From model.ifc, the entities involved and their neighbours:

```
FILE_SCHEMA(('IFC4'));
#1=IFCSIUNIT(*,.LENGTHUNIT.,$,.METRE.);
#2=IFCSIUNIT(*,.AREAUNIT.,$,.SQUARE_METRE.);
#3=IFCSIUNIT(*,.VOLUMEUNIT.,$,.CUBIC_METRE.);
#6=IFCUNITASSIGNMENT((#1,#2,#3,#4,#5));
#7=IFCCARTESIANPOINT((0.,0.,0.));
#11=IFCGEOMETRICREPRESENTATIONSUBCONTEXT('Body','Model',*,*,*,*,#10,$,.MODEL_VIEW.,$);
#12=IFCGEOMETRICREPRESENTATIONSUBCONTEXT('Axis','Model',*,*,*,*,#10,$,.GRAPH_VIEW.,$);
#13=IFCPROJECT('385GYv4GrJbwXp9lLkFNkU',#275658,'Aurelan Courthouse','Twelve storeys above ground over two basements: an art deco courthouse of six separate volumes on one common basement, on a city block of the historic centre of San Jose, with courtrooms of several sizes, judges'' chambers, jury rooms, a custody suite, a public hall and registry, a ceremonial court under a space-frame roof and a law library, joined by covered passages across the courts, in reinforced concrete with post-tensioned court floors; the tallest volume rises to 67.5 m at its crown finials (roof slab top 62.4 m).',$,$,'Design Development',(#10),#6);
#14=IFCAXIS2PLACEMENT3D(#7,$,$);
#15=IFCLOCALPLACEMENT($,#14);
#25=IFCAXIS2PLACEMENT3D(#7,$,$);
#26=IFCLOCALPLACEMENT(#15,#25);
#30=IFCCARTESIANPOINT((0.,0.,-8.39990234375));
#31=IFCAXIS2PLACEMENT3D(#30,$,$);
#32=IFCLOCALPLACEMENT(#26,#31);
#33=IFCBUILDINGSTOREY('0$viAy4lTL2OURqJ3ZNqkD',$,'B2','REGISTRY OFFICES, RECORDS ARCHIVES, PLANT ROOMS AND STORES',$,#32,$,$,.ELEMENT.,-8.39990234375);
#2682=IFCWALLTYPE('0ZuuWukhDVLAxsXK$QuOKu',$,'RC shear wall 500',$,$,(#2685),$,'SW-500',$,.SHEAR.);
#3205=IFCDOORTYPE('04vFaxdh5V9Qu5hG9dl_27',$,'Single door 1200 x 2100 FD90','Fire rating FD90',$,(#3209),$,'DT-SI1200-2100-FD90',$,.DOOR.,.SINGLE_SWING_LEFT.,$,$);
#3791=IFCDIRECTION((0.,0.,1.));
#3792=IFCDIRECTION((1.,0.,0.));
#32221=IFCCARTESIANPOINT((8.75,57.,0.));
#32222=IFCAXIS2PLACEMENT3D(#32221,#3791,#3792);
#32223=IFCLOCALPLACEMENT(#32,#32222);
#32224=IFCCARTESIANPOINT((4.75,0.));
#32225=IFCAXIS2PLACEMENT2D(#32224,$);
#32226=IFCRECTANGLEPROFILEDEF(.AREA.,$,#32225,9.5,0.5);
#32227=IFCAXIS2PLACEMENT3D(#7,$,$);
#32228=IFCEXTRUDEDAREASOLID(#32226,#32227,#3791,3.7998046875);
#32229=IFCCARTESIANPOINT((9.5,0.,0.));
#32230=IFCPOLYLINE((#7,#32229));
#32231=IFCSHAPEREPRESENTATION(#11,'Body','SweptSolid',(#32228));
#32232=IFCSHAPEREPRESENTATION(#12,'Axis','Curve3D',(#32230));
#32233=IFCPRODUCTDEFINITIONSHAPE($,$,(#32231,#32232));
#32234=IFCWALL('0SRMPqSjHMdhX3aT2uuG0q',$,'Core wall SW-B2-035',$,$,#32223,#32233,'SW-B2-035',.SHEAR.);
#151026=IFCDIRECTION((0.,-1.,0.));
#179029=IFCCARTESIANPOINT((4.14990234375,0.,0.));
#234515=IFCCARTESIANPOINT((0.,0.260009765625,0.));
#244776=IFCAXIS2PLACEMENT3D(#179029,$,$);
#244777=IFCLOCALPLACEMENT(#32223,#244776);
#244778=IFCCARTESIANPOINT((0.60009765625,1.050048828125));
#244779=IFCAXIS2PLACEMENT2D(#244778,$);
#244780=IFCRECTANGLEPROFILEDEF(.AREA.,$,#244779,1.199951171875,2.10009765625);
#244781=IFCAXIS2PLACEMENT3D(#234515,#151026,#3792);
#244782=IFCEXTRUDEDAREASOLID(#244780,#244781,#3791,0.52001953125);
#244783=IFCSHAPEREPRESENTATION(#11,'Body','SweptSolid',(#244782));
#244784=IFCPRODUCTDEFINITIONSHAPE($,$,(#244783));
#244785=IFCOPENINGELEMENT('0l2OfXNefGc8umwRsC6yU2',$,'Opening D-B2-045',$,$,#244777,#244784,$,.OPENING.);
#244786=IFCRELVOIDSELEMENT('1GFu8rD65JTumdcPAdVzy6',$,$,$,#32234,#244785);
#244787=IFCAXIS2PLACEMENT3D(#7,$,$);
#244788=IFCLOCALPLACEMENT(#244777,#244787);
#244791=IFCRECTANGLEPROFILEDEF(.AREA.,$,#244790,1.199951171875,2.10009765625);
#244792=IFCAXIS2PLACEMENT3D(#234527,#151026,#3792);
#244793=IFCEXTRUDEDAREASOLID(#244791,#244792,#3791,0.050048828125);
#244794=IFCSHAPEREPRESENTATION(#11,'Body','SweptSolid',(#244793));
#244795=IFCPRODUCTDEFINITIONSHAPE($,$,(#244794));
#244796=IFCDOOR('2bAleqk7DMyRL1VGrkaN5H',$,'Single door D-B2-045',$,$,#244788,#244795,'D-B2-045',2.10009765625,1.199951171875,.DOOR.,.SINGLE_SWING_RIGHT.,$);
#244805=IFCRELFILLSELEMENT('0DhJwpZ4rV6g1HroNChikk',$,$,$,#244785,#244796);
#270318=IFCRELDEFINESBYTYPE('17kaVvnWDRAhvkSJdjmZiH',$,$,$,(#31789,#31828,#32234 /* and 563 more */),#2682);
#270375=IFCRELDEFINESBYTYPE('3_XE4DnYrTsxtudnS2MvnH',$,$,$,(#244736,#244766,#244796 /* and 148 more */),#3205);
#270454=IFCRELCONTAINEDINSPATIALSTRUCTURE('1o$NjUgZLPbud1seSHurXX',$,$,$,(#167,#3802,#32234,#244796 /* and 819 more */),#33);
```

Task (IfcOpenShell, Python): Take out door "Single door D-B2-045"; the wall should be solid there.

```python
import ifcopenshell
import ifcopenshell.api.feature
import ifcopenshell.api.root
import ifcopenshell.geom
import ifcopenshell.util.shape

model = ifcopenshell.open("model.ifc")
settings = ifcopenshell.geom.settings()


def volume(element):
    """Net volume in cubic metres, openings subtracted."""
    shape = ifcopenshell.geom.create_shape(settings, element)
    return ifcopenshell.util.shape.get_volume(shape.geometry)


door = model.by_id(244796)
opening = door.FillsVoids[0].RelatingOpeningElement
wall = opening.VoidsElements[0].RelatingBuildingElement
before = volume(wall)

ifcopenshell.api.root.remove_product(model, product=door)
ifcopenshell.api.feature.remove_feature(model, feature=opening)

after = volume(wall)

print(f"wall volume {before:.3f} -> {after:.3f} m3")

model.write("model-out.ifc")
```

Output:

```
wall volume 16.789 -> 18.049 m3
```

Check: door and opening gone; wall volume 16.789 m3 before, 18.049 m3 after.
